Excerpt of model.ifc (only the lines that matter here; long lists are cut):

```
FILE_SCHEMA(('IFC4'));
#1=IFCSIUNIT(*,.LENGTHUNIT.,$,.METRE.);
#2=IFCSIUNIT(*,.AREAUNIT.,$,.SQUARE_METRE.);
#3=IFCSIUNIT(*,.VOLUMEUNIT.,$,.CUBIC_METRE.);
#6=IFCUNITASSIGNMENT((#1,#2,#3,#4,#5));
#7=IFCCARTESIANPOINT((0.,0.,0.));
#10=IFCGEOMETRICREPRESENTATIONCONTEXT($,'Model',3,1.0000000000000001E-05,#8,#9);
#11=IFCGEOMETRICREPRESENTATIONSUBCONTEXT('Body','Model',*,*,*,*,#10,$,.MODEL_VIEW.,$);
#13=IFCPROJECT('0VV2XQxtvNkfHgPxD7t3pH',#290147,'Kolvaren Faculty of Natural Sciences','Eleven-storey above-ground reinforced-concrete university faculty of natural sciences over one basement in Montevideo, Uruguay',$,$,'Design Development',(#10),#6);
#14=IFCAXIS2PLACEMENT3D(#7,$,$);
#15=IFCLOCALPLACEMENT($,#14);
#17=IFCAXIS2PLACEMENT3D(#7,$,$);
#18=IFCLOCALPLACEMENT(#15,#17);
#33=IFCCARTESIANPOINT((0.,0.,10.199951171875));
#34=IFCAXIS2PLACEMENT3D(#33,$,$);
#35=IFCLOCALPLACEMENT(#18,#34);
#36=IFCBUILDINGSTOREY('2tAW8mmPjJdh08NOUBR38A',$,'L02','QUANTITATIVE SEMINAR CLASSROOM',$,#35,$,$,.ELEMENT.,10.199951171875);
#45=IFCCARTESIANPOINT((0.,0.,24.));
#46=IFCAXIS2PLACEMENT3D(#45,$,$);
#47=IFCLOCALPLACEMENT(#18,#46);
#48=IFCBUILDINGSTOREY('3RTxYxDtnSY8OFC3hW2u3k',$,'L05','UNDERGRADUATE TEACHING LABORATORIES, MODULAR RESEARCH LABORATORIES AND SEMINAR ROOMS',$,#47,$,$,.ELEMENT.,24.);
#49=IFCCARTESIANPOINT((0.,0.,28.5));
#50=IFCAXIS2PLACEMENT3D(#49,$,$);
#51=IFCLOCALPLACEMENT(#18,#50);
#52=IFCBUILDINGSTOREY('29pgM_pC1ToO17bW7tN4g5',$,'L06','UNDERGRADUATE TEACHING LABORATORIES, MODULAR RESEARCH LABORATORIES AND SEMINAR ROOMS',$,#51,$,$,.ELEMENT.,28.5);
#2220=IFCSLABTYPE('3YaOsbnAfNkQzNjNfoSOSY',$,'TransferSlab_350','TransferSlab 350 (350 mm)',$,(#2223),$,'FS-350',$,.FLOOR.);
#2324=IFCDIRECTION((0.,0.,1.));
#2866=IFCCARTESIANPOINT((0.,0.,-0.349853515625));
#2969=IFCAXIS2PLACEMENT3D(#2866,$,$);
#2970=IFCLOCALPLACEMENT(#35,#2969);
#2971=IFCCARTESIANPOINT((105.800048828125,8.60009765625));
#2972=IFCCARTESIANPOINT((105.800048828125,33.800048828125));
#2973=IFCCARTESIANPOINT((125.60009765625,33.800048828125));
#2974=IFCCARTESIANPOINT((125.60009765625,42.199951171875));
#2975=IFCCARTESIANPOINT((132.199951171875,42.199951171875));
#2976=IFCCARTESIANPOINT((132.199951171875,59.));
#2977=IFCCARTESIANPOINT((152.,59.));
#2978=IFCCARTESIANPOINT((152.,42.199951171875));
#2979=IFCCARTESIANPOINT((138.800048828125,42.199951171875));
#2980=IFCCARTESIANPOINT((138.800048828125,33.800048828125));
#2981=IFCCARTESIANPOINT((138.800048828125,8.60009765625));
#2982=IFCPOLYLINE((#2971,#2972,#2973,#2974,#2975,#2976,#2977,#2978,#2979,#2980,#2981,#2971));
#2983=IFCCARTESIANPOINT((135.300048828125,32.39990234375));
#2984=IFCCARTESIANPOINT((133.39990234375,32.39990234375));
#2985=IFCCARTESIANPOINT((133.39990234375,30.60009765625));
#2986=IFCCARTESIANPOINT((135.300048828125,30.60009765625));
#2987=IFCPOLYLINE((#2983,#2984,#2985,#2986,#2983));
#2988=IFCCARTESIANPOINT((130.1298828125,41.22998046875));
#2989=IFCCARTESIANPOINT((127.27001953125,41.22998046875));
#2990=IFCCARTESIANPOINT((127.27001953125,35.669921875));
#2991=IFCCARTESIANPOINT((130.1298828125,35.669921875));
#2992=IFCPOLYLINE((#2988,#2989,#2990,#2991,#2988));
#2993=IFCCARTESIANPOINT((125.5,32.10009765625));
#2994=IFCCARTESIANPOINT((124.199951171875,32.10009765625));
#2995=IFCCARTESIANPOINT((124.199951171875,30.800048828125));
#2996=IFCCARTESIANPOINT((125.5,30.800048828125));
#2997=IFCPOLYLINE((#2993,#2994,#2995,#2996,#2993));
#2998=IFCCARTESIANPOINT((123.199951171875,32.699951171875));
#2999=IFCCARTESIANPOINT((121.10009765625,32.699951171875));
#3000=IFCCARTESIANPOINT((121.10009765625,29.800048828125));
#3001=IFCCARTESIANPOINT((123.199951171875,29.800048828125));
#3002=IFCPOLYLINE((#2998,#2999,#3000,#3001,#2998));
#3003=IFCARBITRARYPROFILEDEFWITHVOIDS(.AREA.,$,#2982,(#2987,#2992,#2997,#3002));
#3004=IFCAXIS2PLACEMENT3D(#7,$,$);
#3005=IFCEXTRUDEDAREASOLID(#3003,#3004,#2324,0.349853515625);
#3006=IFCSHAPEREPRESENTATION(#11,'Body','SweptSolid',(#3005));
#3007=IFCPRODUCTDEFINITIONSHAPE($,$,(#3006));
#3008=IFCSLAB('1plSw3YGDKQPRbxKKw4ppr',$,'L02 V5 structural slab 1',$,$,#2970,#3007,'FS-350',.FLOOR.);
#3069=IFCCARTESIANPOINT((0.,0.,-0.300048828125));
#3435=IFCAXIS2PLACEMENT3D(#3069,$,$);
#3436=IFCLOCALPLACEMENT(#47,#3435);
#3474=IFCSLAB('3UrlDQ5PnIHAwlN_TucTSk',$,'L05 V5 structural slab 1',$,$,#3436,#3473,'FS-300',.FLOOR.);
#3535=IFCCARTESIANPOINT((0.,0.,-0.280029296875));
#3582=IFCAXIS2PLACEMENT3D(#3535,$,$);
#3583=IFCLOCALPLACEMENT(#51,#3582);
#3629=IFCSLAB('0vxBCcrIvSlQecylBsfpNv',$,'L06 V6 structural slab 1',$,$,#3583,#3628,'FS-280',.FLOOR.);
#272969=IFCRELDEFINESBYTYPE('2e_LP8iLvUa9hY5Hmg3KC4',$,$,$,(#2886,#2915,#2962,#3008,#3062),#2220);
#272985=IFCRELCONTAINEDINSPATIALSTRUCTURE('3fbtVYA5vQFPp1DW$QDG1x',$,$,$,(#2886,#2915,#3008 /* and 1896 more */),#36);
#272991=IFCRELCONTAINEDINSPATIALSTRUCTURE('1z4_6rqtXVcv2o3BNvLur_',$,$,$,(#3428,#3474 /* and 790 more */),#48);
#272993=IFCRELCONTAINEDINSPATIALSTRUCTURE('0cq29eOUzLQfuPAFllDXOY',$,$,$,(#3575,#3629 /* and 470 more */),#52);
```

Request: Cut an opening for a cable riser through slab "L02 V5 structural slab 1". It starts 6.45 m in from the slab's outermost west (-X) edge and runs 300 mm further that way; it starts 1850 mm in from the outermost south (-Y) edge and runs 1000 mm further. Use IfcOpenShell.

```python
import numpy as np
import ifcopenshell
import ifcopenshell.api.feature
import ifcopenshell.api.geometry
import ifcopenshell.api.root
import ifcopenshell.geom
import ifcopenshell.util.placement
import ifcopenshell.util.representation
import ifcopenshell.util.shape
import ifcopenshell.util.unit

model = ifcopenshell.open("model.ifc")
unit_scale = ifcopenshell.util.unit.calculate_unit_scale(model)
settings = ifcopenshell.geom.settings()


def volume(element):
    """Net volume in cubic metres, openings subtracted."""
    shape = ifcopenshell.geom.create_shape(settings, element)
    return ifcopenshell.util.shape.get_volume(shape.geometry)


slab = model.by_id(3008)
before = volume(slab)

# Extent in the slab's own axes, in metres. The edges named are its -X and -Y sides.
slab_shape = ifcopenshell.geom.create_shape(settings, slab)
vertices = ifcopenshell.util.shape.get_vertices(slab_shape.geometry)
x_min, y_min, bottom = vertices.min(axis=0)
top = vertices[:, 2].max()

opening = ifcopenshell.api.root.create_entity(model, ifc_class="IfcOpeningElement", name="Cable riser opening", predefined_type="OPENING")
context = ifcopenshell.util.representation.get_context(model, "Model", "Body", "MODEL_VIEW")
width, depth = 0.3, 1
outline = [(0.0, 0.0), (width, 0.0), (width, depth), (0.0, depth), (0.0, 0.0)]
# Overshoot both faces by 50 mm so the cut is clean.
shape = ifcopenshell.api.geometry.add_slab_representation(
    model, context=context, depth=top - bottom + 0.1, polyline=outline
)
ifcopenshell.api.geometry.assign_representation(model, product=opening, representation=shape)

matrix = ifcopenshell.util.placement.get_local_placement(slab.ObjectPlacement)
matrix[:, 3] = matrix @ np.append(np.array([x_min + 6.45, y_min + 1.85, bottom - 0.05]) / unit_scale, 1.0)
ifcopenshell.api.geometry.edit_object_placement(model, product=opening, matrix=matrix, is_si=False)
ifcopenshell.api.feature.add_feature(model, feature=opening, element=slab)

after = volume(slab)

print(f"slab volume {before:.3f} -> {after:.3f} m3")

model.write("model-out.ifc")
```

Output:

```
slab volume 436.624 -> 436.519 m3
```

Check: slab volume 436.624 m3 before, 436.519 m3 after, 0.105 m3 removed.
